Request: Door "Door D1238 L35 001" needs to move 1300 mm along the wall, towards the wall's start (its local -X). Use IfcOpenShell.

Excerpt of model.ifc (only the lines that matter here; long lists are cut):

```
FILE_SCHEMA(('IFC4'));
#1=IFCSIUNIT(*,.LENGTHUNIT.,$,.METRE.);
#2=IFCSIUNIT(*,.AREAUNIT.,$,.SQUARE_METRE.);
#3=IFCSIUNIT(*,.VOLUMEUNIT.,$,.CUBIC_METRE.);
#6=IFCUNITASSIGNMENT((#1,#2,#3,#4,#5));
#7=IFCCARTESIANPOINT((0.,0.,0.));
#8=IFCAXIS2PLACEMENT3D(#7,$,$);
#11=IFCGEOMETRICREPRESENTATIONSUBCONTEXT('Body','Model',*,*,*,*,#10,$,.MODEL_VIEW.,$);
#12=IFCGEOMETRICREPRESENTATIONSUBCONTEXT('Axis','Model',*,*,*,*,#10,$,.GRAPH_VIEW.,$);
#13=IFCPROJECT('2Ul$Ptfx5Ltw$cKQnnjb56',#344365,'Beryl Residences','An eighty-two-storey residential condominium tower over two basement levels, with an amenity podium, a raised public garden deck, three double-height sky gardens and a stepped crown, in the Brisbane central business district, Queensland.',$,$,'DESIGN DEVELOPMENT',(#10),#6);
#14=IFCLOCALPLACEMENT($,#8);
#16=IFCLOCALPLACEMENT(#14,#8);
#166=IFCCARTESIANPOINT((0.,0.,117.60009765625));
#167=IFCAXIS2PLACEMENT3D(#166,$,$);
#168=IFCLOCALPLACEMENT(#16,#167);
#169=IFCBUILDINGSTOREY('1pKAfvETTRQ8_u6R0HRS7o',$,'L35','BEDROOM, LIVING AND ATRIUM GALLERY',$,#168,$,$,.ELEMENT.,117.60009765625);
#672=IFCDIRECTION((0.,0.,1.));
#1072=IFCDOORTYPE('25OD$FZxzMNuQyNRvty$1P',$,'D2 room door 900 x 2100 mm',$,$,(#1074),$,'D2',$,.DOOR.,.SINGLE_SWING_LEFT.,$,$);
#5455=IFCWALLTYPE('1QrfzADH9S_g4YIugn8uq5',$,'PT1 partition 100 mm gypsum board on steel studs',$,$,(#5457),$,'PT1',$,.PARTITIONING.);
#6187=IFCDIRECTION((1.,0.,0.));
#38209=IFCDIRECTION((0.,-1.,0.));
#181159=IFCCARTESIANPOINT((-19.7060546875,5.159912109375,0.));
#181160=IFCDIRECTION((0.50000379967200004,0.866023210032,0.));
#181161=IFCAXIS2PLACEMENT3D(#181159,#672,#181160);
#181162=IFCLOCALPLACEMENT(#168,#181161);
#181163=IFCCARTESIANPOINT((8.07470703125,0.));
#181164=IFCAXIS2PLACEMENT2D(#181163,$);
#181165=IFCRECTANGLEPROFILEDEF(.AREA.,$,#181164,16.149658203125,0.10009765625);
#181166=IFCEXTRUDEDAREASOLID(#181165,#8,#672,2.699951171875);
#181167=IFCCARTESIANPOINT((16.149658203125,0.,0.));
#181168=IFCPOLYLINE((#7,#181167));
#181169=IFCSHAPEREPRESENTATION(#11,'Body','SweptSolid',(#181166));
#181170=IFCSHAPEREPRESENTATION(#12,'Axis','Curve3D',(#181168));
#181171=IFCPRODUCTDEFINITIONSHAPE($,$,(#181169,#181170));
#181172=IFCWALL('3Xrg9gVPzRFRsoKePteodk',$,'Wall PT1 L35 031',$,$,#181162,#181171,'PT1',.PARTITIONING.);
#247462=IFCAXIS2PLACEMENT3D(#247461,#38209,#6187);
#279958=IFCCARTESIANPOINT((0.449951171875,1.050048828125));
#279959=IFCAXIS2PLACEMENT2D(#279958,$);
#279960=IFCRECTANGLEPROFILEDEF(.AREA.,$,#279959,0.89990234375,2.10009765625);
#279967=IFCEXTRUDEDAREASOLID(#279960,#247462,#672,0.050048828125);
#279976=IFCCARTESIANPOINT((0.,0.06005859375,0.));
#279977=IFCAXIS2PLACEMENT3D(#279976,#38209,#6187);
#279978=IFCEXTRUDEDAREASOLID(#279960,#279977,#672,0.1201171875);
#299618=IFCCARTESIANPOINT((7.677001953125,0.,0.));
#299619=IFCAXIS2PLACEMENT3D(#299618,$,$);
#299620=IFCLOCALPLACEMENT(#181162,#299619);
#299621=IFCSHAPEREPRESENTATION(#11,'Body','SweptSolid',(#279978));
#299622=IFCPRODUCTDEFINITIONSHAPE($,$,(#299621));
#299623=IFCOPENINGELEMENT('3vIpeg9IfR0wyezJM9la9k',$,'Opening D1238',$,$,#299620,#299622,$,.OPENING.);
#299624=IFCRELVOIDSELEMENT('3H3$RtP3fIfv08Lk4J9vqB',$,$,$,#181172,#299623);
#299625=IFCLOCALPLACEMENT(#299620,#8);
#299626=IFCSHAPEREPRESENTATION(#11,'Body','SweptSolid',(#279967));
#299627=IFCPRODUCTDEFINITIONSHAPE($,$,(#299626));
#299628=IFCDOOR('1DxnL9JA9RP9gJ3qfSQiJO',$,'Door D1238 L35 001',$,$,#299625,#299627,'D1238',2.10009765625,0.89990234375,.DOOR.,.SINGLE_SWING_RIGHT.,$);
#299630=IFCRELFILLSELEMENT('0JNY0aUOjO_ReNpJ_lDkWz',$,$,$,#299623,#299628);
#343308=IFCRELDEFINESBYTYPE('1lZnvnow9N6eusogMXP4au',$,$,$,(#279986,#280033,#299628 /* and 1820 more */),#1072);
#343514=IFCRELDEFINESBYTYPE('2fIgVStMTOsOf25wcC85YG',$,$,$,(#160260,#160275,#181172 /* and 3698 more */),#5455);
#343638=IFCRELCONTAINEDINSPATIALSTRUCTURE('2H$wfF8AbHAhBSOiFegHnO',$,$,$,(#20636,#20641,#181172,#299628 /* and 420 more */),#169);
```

```python
import ifcopenshell
import ifcopenshell.api.geometry
import ifcopenshell.util.placement
import ifcopenshell.util.unit

model = ifcopenshell.open("model.ifc")
unit_scale = ifcopenshell.util.unit.calculate_unit_scale(model)

door = model.by_guid("1DxnL9JA9RP9gJ3qfSQiJO")
opening = door.FillsVoids[0].RelatingOpeningElement
wall = opening.VoidsElements[0].RelatingBuildingElement

wall_matrix = ifcopenshell.util.placement.get_local_placement(wall.ObjectPlacement)
shift = wall_matrix[:3, 0] * -1.3 / unit_scale
before = ifcopenshell.util.placement.get_local_placement(door.ObjectPlacement)[:3, 3].copy()

# The door is placed relative to its opening, so it follows when the opening moves.
matrix = ifcopenshell.util.placement.get_local_placement(opening.ObjectPlacement)
matrix[:3, 3] += shift
ifcopenshell.api.geometry.edit_object_placement(
    model, product=opening, matrix=matrix, is_si=False, should_transform_children=True
)

after = ifcopenshell.util.placement.get_local_placement(door.ObjectPlacement)[:3, 3]
print("door moved by", (after - before).round(3) + 0.0)

model.write("model_updated.ifc")
```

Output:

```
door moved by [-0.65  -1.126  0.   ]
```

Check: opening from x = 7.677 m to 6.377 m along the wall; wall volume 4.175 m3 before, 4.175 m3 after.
